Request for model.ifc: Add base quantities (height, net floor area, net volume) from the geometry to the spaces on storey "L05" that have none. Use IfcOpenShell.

First a look at what the model holds.

```python
import ifcopenshell
import ifcopenshell.util.element
import ifcopenshell.util.unit

model = ifcopenshell.open("model.ifc")
print(model.schema)
for unit_type in ("LENGTHUNIT", "AREAUNIT", "VOLUMEUNIT"):
    print(unit_type, ifcopenshell.util.unit.calculate_unit_scale(model, unit_type))
storey = next(s for s in model.by_type("IfcBuildingStorey") if s.Name == "L05")
spaces = [e for e in ifcopenshell.util.element.get_decomposition(storey) if e.is_a("IfcSpace")]
for e in sorted(spaces, key=lambda e: e.id()):
    print(e.id(), e.is_a(), e.Name, list(ifcopenshell.util.element.get_psets(e, qtos_only=True)), sep=" | ")
```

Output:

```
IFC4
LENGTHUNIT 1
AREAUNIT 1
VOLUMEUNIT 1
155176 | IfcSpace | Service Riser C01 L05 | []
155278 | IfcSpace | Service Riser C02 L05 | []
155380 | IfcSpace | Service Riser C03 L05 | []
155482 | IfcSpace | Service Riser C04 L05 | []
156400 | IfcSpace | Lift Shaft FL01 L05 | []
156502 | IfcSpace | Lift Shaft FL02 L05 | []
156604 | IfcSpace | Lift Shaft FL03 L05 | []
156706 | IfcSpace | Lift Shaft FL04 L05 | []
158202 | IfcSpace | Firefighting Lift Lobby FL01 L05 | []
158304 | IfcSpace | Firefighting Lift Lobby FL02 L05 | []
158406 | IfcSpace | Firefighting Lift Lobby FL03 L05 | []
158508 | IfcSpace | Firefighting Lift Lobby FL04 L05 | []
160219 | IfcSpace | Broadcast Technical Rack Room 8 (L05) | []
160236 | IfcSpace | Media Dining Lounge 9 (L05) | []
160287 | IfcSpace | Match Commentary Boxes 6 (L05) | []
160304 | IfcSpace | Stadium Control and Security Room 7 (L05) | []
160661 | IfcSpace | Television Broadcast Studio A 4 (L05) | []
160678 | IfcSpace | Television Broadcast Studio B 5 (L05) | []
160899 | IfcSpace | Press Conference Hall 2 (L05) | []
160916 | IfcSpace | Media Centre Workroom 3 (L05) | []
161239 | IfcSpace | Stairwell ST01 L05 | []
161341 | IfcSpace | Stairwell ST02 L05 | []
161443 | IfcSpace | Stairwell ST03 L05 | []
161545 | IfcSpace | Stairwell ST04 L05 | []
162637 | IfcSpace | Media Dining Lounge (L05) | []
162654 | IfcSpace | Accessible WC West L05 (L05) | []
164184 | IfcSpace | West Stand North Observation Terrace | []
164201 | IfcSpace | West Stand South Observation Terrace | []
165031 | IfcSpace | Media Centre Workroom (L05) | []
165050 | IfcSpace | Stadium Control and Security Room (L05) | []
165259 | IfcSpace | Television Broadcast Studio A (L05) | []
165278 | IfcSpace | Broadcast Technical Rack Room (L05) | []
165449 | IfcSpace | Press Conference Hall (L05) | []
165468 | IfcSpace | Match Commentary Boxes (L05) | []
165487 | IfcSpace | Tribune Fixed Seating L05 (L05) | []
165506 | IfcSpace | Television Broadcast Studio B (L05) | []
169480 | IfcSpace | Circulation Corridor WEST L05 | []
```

```python
import ifcopenshell
import ifcopenshell.api.pset
import ifcopenshell.geom
import ifcopenshell.util.element
import ifcopenshell.util.shape
import ifcopenshell.util.unit

model = ifcopenshell.open("model.ifc")
unit_scale = ifcopenshell.util.unit.calculate_unit_scale(model)
area_scale = ifcopenshell.util.unit.calculate_unit_scale(model, "AREAUNIT")
volume_scale = ifcopenshell.util.unit.calculate_unit_scale(model, "VOLUMEUNIT")
settings = ifcopenshell.geom.settings()

storey = next(s for s in model.by_type("IfcBuildingStorey") if s.Name == "L05")
spaces = [e for e in ifcopenshell.util.element.get_decomposition(storey) if e.is_a("IfcSpace")]

for e in sorted(spaces, key=lambda e: e.id()):
    if ifcopenshell.util.element.get_psets(e, qtos_only=True, should_inherit=False):
        continue
    # Geometry comes back in metres, in the element's own axes.
    shape = ifcopenshell.geom.create_shape(settings, e)
    values = {
        "Height": ifcopenshell.util.shape.get_z(shape.geometry) / unit_scale,
        "NetFloorArea": ifcopenshell.util.shape.get_footprint_area(shape.geometry) / area_scale,
        "NetVolume": ifcopenshell.util.shape.get_volume(shape.geometry) / volume_scale,
    }
    qto = ifcopenshell.api.pset.add_qto(model, product=e, name="Qto_SpaceBaseQuantities")
    ifcopenshell.api.pset.edit_qto(model, qto=qto, properties=values)
    print(e.id(), {k: round(v, 3) for k, v in values.items()})

model.write("model_v2.ifc")
```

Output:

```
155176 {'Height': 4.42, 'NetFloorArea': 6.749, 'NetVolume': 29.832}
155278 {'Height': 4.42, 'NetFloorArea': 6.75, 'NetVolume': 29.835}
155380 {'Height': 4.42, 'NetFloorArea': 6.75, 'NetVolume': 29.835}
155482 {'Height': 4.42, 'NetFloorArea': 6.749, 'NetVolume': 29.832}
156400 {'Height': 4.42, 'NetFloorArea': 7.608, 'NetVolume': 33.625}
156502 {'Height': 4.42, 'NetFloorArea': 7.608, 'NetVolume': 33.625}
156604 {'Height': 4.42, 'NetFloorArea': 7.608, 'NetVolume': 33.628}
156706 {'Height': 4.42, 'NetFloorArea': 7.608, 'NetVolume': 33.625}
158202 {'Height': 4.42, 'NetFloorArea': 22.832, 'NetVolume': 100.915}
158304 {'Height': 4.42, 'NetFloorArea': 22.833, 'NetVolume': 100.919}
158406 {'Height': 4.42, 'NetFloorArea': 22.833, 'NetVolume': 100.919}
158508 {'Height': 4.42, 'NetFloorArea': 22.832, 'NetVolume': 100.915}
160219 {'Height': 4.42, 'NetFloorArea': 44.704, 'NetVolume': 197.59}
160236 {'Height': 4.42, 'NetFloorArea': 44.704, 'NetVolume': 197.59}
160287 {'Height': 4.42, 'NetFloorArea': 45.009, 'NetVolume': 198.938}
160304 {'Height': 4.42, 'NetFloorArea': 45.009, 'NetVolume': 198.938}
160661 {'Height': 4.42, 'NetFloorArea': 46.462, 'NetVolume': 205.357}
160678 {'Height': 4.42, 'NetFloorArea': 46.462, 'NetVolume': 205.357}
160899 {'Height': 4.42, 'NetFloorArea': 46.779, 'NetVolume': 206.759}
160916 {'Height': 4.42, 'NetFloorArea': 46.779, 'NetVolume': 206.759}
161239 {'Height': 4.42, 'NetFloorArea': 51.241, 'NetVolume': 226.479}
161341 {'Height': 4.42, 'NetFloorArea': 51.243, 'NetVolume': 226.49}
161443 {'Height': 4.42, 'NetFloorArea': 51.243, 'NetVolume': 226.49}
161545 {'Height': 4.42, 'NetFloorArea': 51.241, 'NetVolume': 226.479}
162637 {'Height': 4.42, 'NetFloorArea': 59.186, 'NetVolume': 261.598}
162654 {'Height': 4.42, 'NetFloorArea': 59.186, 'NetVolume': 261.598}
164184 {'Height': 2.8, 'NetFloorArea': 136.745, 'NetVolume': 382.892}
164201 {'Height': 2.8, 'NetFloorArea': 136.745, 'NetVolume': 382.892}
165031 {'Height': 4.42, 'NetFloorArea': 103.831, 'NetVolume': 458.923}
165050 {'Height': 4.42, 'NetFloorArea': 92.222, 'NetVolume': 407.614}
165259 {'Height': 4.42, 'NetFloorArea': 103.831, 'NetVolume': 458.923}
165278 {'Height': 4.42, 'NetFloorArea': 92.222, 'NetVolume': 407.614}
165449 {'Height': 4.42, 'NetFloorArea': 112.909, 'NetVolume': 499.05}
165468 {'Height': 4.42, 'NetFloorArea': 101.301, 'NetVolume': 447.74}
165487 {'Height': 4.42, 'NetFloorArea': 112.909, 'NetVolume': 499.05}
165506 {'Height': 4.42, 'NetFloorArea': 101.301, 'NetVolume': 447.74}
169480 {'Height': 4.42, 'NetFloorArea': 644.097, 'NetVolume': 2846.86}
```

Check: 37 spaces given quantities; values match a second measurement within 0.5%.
